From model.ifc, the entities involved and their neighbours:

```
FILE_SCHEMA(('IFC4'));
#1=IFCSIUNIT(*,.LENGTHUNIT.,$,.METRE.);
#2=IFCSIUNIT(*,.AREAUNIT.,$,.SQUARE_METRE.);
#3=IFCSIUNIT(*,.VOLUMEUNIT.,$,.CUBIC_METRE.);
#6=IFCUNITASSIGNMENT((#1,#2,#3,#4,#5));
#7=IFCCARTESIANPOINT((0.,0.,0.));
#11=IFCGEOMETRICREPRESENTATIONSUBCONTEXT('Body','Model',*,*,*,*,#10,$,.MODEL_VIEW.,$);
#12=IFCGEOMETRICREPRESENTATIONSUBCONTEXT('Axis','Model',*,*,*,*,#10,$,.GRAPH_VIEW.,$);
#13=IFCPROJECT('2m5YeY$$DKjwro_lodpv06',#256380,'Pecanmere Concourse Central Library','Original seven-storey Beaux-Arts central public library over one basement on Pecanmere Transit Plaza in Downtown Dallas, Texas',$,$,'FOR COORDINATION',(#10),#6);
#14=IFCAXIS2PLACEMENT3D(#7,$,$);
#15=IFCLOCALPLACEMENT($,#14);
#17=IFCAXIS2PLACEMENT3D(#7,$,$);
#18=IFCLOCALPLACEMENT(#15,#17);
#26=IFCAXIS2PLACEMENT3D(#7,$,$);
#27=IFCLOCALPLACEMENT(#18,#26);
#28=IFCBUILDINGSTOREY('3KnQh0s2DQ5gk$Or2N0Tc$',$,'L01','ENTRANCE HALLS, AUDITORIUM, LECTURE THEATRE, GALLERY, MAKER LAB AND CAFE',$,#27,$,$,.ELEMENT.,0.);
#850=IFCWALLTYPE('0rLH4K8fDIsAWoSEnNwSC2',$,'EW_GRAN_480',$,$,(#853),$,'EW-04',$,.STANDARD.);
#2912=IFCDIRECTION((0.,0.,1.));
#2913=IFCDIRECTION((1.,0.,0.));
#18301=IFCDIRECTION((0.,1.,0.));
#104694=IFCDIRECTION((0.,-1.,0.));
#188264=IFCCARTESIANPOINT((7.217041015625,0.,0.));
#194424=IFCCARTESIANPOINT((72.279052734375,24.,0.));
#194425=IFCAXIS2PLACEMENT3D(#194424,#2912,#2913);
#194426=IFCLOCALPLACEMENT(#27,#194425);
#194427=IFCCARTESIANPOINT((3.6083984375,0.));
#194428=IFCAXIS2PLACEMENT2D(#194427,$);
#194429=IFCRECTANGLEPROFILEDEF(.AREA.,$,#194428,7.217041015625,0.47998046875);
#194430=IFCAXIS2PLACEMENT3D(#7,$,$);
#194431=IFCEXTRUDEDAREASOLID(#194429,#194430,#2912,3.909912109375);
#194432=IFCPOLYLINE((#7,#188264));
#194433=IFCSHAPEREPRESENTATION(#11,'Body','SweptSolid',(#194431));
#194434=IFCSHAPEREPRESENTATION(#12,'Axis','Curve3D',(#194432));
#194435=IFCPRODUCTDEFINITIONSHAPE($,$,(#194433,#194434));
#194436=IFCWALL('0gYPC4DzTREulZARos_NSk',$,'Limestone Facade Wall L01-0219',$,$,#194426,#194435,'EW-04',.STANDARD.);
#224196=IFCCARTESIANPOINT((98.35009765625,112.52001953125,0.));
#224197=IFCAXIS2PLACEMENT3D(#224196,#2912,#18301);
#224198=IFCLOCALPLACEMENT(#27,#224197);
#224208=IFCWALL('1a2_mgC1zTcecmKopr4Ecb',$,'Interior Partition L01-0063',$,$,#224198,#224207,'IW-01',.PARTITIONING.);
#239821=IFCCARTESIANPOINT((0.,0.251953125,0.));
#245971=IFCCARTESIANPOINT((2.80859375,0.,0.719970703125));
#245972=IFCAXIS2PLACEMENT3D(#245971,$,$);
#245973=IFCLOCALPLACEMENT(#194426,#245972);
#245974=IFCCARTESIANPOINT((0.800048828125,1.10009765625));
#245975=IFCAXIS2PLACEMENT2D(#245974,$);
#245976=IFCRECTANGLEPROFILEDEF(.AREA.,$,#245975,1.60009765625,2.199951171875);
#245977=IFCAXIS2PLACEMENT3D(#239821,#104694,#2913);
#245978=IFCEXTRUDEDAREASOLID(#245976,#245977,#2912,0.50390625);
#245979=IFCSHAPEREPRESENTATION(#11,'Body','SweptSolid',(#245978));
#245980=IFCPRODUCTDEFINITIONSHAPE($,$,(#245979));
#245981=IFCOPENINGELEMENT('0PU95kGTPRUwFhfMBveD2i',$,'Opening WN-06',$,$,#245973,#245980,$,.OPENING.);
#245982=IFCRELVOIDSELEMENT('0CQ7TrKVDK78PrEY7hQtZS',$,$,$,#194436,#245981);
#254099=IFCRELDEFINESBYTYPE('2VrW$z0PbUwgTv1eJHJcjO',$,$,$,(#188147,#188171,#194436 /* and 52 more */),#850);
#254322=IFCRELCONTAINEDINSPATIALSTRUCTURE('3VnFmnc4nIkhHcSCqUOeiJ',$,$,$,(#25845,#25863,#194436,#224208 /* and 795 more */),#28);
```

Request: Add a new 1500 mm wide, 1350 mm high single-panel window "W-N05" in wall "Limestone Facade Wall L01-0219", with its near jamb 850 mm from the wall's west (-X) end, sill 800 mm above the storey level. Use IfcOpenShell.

```python
import numpy as np
import ifcopenshell
import ifcopenshell.api.feature
import ifcopenshell.api.geometry
import ifcopenshell.api.root
import ifcopenshell.api.spatial
import ifcopenshell.geom
import ifcopenshell.util.element
import ifcopenshell.util.placement
import ifcopenshell.util.representation
import ifcopenshell.util.shape
import ifcopenshell.util.unit

model = ifcopenshell.open("model.ifc")
unit_scale = ifcopenshell.util.unit.calculate_unit_scale(model)
settings = ifcopenshell.geom.settings()


def volume(element):
    """Net volume in cubic metres, openings subtracted."""
    shape = ifcopenshell.geom.create_shape(settings, element)
    return ifcopenshell.util.shape.get_volume(shape.geometry)


wall = model.by_id(194436)
storey = ifcopenshell.util.element.get_container(wall, ifc_class="IfcBuildingStorey")
context = ifcopenshell.util.representation.get_context(model, "Model", "Body", "MODEL_VIEW")
before = volume(wall)

width, height, from_end, sill = 1.5, 1.35, 0.85, 0.8  # metres

# The wall runs along its own X axis, and the end named is its -X end.
wall_shape = ifcopenshell.geom.create_shape(settings, wall)
x, y, z = ifcopenshell.util.shape.get_vertices(wall_shape.geometry).T
start = x.min() + from_end
face, thickness = float(y.min()), float(y.max() - y.min())
wall_matrix = ifcopenshell.util.placement.get_local_placement(wall.ObjectPlacement)
level = ifcopenshell.util.placement.get_local_placement(storey.ObjectPlacement)[2, 3]


def in_wall(x, y):
    """Placement at x, y metres in the wall's axes, at sill height."""
    matrix = wall_matrix.copy()
    matrix[:, 3] = wall_matrix @ np.array([x / unit_scale, y / unit_scale, 0.0, 1.0])
    matrix[2, 3] = level + sill / unit_scale
    return matrix


# Opening: a box that overshoots both wall faces by 50 mm.
opening = ifcopenshell.api.root.create_entity(model, ifc_class="IfcOpeningElement", predefined_type="OPENING")
box = ifcopenshell.api.geometry.add_wall_representation(
    model, context=context, length=width, height=height, thickness=thickness + 0.1
)
ifcopenshell.api.geometry.assign_representation(model, product=opening, representation=box)
ifcopenshell.api.geometry.edit_object_placement(model, product=opening, matrix=in_wall(start, face - 0.05), is_si=False)
ifcopenshell.api.feature.add_feature(model, feature=opening, element=wall)

window = ifcopenshell.api.root.create_entity(model, ifc_class="IfcWindow", name="W-N05", predefined_type="WINDOW")
window.OverallWidth, window.OverallHeight = width / unit_scale, height / unit_scale
window.PartitioningType = "SINGLE_PANEL"
body = ifcopenshell.api.geometry.add_window_representation(
    model,
    context=context,
    overall_width=window.OverallWidth,
    overall_height=window.OverallHeight,
    partition_type="SINGLE_PANEL",
)
ifcopenshell.api.geometry.assign_representation(model, product=window, representation=body)
ifcopenshell.api.spatial.assign_container(model, products=[window], relating_structure=storey)
ifcopenshell.api.feature.add_filling(model, opening=opening, element=window)

# Centre the window in the wall's thickness.
ifcopenshell.api.geometry.edit_object_placement(model, product=window, matrix=in_wall(start, face), is_si=False)
window_shape = ifcopenshell.geom.create_shape(settings, window)
depth = ifcopenshell.util.shape.get_vertices(window_shape.geometry)[:, 1]
offset = face + thickness / 2 - (depth.min() + depth.max()) / 2
ifcopenshell.api.geometry.edit_object_placement(model, product=window, matrix=in_wall(start, offset), is_si=False)

after = volume(wall)

print(f"wall volume {before:.3f} -> {after:.3f} m3")

model.write("model_edited.ifc")
```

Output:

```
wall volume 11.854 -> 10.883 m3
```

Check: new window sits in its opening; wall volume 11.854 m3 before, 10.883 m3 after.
